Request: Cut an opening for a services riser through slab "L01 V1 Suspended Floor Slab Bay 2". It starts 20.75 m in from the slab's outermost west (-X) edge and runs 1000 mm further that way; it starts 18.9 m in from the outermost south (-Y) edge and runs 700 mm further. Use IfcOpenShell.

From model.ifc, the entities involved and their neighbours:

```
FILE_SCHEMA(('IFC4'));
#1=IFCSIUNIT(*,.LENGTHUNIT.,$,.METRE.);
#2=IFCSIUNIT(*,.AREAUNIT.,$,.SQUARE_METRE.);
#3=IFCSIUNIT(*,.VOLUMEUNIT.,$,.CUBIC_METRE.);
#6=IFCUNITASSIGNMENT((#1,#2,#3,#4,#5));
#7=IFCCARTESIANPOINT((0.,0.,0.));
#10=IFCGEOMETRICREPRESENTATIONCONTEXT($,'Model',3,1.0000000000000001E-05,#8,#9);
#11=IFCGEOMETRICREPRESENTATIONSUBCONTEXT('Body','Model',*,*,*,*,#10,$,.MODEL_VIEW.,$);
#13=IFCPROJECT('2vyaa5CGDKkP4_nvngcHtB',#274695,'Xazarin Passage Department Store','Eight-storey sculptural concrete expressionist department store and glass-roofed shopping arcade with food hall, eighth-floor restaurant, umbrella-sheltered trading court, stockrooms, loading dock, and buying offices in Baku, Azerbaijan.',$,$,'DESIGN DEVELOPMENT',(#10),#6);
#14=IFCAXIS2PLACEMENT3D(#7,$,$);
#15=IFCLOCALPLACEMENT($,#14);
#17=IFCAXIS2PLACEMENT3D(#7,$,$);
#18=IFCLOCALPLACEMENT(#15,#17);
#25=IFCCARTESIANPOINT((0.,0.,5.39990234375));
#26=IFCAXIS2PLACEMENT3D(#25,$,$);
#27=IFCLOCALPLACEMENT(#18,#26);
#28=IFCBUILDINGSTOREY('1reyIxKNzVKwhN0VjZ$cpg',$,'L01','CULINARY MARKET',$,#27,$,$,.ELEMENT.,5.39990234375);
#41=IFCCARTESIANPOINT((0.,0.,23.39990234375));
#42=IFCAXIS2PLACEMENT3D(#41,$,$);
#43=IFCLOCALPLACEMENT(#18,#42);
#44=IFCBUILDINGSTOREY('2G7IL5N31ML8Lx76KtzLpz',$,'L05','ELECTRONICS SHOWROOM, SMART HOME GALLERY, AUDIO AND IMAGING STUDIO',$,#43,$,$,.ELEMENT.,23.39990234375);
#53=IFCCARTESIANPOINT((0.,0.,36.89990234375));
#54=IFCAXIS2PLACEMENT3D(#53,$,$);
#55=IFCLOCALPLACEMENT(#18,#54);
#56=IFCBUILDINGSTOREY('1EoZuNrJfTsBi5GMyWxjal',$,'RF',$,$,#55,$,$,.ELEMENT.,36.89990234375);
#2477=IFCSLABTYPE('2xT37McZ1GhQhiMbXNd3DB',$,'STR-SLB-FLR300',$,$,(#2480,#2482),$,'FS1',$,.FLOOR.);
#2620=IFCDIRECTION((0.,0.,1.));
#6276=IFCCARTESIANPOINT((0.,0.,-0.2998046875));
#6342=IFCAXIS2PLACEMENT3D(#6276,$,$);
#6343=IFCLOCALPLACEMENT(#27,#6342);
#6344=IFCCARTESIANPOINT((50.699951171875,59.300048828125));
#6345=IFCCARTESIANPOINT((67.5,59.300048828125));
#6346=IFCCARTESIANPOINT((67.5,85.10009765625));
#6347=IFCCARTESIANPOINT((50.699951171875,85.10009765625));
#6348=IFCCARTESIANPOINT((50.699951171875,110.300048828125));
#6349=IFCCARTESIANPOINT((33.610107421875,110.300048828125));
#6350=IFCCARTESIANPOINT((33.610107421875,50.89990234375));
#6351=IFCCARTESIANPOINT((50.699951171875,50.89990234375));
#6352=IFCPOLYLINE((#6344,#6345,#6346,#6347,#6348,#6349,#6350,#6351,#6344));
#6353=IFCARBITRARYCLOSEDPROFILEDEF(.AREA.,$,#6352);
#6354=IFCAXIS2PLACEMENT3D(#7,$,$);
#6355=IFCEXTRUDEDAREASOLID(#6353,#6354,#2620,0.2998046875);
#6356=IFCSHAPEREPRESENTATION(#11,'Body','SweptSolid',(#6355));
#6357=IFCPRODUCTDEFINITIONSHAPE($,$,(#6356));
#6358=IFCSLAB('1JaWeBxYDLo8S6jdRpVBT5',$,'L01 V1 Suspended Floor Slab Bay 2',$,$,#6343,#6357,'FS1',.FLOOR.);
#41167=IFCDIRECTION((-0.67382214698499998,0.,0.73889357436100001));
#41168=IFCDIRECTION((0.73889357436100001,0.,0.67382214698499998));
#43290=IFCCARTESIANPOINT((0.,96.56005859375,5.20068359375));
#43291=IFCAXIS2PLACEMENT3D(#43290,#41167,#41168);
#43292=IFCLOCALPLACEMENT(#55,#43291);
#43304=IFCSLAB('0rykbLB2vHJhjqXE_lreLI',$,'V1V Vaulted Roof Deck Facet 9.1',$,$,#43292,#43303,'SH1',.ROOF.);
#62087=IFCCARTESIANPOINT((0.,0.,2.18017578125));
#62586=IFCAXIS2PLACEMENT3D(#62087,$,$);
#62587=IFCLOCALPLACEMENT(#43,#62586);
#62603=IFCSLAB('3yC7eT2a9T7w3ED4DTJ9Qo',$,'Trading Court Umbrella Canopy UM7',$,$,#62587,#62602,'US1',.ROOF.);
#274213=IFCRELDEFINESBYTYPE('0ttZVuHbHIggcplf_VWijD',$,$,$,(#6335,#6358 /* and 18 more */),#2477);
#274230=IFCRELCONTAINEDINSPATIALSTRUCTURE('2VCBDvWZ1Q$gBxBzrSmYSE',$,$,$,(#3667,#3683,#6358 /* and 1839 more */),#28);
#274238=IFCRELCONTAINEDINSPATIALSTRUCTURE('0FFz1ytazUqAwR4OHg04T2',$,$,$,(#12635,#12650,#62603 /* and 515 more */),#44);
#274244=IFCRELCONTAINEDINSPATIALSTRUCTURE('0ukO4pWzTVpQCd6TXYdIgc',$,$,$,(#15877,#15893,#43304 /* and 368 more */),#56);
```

```python
import numpy as np
import ifcopenshell
import ifcopenshell.api.feature
import ifcopenshell.api.geometry
import ifcopenshell.api.root
import ifcopenshell.geom
import ifcopenshell.util.placement
import ifcopenshell.util.representation
import ifcopenshell.util.shape
import ifcopenshell.util.unit

model = ifcopenshell.open("model.ifc")
unit_scale = ifcopenshell.util.unit.calculate_unit_scale(model)
settings = ifcopenshell.geom.settings()


def volume(element):
    """Net volume in cubic metres, openings subtracted."""
    shape = ifcopenshell.geom.create_shape(settings, element)
    return ifcopenshell.util.shape.get_volume(shape.geometry)


slab = model.by_guid("1JaWeBxYDLo8S6jdRpVBT5")
before = volume(slab)

# Extent in the slab's own axes, in metres. The edges named are its -X and -Y sides.
slab_shape = ifcopenshell.geom.create_shape(settings, slab)
vertices = ifcopenshell.util.shape.get_vertices(slab_shape.geometry)
x_min, y_min, bottom = vertices.min(axis=0)
top = vertices[:, 2].max()

opening = ifcopenshell.api.root.create_entity(model, ifc_class="IfcOpeningElement", name="Services riser opening", predefined_type="OPENING")
context = ifcopenshell.util.representation.get_context(model, "Model", "Body", "MODEL_VIEW")
width, depth = 1, 0.7
outline = [(0.0, 0.0), (width, 0.0), (width, depth), (0.0, depth), (0.0, 0.0)]
# Overshoot both faces by 50 mm so the cut is clean.
shape = ifcopenshell.api.geometry.add_slab_representation(
    model, context=context, depth=top - bottom + 0.1, polyline=outline
)
ifcopenshell.api.geometry.assign_representation(model, product=opening, representation=shape)

matrix = ifcopenshell.util.placement.get_local_placement(slab.ObjectPlacement)
matrix[:, 3] = matrix @ np.append(np.array([x_min + 20.75, y_min + 18.9, bottom - 0.05]) / unit_scale, 1.0)
ifcopenshell.api.geometry.edit_object_placement(model, product=opening, matrix=matrix, is_si=False)
ifcopenshell.api.feature.add_feature(model, feature=opening, element=slab)

after = volume(slab)

print(f"slab volume {before:.3f} -> {after:.3f} m3")

model.write("model_edited.ifc")
```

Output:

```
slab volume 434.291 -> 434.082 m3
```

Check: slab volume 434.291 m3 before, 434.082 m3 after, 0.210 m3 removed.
